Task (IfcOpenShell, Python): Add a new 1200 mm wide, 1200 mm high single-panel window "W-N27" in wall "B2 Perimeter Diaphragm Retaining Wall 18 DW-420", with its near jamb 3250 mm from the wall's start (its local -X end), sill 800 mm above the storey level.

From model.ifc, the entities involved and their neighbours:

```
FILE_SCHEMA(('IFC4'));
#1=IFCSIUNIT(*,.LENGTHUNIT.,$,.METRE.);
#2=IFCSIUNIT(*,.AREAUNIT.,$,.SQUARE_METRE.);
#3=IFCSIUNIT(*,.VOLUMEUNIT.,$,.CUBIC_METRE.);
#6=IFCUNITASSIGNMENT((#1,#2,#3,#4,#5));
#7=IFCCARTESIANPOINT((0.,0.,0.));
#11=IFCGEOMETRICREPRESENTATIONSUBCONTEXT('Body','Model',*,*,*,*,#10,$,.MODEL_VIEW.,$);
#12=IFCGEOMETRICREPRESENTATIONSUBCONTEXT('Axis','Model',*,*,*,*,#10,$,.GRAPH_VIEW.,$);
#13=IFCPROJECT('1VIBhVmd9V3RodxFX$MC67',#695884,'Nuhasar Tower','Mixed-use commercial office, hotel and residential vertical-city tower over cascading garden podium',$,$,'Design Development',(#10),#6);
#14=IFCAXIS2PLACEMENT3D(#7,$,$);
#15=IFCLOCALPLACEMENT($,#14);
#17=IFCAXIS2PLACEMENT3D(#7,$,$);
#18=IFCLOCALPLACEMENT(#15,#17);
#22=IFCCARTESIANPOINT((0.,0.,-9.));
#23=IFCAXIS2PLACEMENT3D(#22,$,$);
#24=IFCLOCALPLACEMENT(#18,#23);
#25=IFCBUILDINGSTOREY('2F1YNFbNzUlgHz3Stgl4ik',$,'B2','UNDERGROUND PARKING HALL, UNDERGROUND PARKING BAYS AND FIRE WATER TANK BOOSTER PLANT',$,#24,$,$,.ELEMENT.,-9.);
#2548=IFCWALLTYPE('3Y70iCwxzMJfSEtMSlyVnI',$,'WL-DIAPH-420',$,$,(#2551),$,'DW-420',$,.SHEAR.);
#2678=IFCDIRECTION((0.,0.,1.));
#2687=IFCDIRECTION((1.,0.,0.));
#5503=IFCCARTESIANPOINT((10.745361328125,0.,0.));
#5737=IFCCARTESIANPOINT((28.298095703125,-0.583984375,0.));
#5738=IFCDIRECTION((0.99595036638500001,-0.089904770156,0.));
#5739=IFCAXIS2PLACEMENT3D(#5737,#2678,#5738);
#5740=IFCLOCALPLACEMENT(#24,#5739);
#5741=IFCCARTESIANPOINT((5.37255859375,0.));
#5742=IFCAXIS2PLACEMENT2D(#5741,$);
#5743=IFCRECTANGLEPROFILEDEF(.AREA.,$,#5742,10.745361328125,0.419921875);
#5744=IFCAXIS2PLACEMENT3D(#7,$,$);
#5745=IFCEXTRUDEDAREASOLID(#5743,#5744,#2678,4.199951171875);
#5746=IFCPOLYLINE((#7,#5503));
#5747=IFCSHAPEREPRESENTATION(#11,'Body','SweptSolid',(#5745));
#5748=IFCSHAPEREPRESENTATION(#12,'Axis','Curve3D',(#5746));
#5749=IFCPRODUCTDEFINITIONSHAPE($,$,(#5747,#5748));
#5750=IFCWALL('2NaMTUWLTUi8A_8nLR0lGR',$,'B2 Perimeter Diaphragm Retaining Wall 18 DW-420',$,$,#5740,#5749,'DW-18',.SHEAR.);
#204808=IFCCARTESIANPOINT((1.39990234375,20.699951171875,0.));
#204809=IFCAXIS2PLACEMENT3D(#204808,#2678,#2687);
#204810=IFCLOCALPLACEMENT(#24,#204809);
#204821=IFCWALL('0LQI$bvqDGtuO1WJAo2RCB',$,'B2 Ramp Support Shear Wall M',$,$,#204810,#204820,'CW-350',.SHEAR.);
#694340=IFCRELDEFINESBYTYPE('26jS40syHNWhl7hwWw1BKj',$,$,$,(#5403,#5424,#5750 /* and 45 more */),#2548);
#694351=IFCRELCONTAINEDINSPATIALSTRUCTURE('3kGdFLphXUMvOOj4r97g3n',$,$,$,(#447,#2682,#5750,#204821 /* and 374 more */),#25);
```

```python
import numpy as np
import ifcopenshell
import ifcopenshell.api.feature
import ifcopenshell.api.geometry
import ifcopenshell.api.root
import ifcopenshell.api.spatial
import ifcopenshell.geom
import ifcopenshell.util.element
import ifcopenshell.util.placement
import ifcopenshell.util.representation
import ifcopenshell.util.shape
import ifcopenshell.util.unit

model = ifcopenshell.open("model.ifc")
unit_scale = ifcopenshell.util.unit.calculate_unit_scale(model)
settings = ifcopenshell.geom.settings()


def volume(element):
    """Net volume in cubic metres, openings subtracted."""
    shape = ifcopenshell.geom.create_shape(settings, element)
    return ifcopenshell.util.shape.get_volume(shape.geometry)


wall = model.by_id(5750)
storey = ifcopenshell.util.element.get_container(wall, ifc_class="IfcBuildingStorey")
context = ifcopenshell.util.representation.get_context(model, "Model", "Body", "MODEL_VIEW")
before = volume(wall)

width, height, from_end, sill = 1.2, 1.2, 3.25, 0.8  # metres

# The wall runs along its own X axis, and the end named is its -X end.
wall_shape = ifcopenshell.geom.create_shape(settings, wall)
x, y, z = ifcopenshell.util.shape.get_vertices(wall_shape.geometry).T
start = x.min() + from_end
face, thickness = float(y.min()), float(y.max() - y.min())
wall_matrix = ifcopenshell.util.placement.get_local_placement(wall.ObjectPlacement)
level = ifcopenshell.util.placement.get_local_placement(storey.ObjectPlacement)[2, 3]


def in_wall(x, y):
    """Placement at x, y metres in the wall's axes, at sill height."""
    matrix = wall_matrix.copy()
    matrix[:, 3] = wall_matrix @ np.array([x / unit_scale, y / unit_scale, 0.0, 1.0])
    matrix[2, 3] = level + sill / unit_scale
    return matrix


# Opening: a box that overshoots both wall faces by 50 mm.
opening = ifcopenshell.api.root.create_entity(model, ifc_class="IfcOpeningElement", predefined_type="OPENING")
box = ifcopenshell.api.geometry.add_wall_representation(
    model, context=context, length=width, height=height, thickness=thickness + 0.1
)
ifcopenshell.api.geometry.assign_representation(model, product=opening, representation=box)
ifcopenshell.api.geometry.edit_object_placement(model, product=opening, matrix=in_wall(start, face - 0.05), is_si=False)
ifcopenshell.api.feature.add_feature(model, feature=opening, element=wall)

window = ifcopenshell.api.root.create_entity(model, ifc_class="IfcWindow", name="W-N27", predefined_type="WINDOW")
window.OverallWidth, window.OverallHeight = width / unit_scale, height / unit_scale
window.PartitioningType = "SINGLE_PANEL"
body = ifcopenshell.api.geometry.add_window_representation(
    model,
    context=context,
    overall_width=window.OverallWidth,
    overall_height=window.OverallHeight,
    partition_type="SINGLE_PANEL",
)
ifcopenshell.api.geometry.assign_representation(model, product=window, representation=body)
ifcopenshell.api.spatial.assign_container(model, products=[window], relating_structure=storey)
ifcopenshell.api.feature.add_filling(model, opening=opening, element=window)

# Centre the window in the wall's thickness.
ifcopenshell.api.geometry.edit_object_placement(model, product=window, matrix=in_wall(start, face), is_si=False)
window_shape = ifcopenshell.geom.create_shape(settings, window)
depth = ifcopenshell.util.shape.get_vertices(window_shape.geometry)[:, 1]
offset = face + thickness / 2 - (depth.min() + depth.max()) / 2
ifcopenshell.api.geometry.edit_object_placement(model, product=window, matrix=in_wall(start, offset), is_si=False)

after = volume(wall)

print(f"wall volume {before:.3f} -> {after:.3f} m3")

model.write("model_v2.ifc")
```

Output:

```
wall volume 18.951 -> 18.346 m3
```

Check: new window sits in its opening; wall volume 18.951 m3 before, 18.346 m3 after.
